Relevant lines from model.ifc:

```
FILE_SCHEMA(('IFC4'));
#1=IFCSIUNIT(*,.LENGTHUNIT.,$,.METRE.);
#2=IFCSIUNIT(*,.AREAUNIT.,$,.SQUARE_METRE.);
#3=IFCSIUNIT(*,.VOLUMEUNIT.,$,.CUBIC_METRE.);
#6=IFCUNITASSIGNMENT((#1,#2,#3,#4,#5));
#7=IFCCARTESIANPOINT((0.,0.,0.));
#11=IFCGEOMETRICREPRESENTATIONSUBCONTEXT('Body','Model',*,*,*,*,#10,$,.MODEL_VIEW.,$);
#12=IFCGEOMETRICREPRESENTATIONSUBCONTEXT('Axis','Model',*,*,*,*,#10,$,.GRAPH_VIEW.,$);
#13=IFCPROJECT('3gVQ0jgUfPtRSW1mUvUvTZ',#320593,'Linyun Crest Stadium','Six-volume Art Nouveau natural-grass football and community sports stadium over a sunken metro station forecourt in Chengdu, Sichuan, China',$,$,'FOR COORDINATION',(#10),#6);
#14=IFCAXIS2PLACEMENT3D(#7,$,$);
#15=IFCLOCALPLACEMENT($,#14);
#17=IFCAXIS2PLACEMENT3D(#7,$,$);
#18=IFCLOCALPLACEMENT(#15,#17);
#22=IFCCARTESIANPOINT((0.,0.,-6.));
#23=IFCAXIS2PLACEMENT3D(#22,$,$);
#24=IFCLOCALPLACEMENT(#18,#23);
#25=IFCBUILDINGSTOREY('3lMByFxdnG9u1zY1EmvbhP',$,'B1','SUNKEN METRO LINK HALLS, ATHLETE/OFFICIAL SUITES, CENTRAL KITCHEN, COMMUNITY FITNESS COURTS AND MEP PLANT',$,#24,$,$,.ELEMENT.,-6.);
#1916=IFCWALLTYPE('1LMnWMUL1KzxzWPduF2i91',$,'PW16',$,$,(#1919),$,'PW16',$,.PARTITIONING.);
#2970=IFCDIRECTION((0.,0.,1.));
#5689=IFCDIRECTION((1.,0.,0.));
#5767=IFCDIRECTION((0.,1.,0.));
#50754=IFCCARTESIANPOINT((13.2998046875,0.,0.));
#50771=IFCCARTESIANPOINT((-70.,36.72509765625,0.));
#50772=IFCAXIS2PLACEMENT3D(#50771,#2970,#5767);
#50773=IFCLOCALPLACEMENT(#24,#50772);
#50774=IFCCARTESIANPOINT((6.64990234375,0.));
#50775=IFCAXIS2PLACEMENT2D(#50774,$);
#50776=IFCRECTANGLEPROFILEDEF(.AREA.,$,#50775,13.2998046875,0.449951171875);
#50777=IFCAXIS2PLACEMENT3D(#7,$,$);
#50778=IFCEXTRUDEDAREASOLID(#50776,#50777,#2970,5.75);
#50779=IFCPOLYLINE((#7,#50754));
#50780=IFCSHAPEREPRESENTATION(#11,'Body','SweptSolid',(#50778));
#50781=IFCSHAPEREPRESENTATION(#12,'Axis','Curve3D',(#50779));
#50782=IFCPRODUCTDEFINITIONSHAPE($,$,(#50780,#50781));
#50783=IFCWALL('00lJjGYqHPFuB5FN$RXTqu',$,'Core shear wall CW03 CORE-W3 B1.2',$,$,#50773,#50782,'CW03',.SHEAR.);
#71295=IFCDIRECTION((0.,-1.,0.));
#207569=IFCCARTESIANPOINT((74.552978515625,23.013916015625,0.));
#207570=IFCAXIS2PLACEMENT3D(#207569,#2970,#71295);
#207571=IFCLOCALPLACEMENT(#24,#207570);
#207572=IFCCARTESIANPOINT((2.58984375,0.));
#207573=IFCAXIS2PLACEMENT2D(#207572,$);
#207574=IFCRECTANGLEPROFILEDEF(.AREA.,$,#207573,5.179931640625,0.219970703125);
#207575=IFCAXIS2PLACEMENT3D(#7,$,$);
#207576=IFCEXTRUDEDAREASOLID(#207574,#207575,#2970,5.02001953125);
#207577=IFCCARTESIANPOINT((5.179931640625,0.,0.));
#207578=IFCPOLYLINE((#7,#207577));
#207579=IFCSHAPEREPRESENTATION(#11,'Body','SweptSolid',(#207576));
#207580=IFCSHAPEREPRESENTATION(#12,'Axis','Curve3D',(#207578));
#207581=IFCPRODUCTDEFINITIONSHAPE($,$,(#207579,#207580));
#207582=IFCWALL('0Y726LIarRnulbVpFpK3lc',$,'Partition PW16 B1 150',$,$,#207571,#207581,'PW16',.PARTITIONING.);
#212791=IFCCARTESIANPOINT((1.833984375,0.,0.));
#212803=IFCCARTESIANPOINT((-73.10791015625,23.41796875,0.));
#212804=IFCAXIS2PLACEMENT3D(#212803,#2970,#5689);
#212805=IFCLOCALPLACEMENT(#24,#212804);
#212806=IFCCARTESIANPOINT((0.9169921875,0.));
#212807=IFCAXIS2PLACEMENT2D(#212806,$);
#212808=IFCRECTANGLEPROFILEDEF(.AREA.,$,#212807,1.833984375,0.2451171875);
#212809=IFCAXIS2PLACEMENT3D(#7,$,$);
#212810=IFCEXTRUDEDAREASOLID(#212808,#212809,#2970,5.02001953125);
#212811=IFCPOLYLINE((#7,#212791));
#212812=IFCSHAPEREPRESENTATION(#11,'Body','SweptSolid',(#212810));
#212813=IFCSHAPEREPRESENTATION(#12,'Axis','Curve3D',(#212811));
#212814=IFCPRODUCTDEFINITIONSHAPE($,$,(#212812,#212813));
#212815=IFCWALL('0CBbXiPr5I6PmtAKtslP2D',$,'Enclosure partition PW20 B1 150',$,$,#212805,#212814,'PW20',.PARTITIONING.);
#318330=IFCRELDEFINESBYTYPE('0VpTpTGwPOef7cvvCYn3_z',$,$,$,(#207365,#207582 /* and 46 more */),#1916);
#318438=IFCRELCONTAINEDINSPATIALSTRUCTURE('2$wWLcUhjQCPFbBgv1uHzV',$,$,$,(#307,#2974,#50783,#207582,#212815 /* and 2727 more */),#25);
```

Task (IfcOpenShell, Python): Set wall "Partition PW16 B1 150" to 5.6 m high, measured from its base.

```python
import ifcopenshell
import ifcopenshell.geom
import ifcopenshell.util.representation
import ifcopenshell.util.shape

model = ifcopenshell.open("model.ifc")
settings = ifcopenshell.geom.settings()


def volume(element):
    """Net volume in cubic metres, openings subtracted."""
    shape = ifcopenshell.geom.create_shape(settings, element)
    return ifcopenshell.util.shape.get_volume(shape.geometry)


wall = model.by_id(207582)
before = volume(wall)

body = ifcopenshell.util.representation.get_representation(wall, "Model", "Body")
solid = body.Items[0]
old_height = solid.Depth
solid.Depth = 5.6
after = volume(wall)

print(f"height {old_height:g} -> {solid.Depth:g}, volume {before:.3f} -> {after:.3f} m3")

model.write("model_v2.ifc")
```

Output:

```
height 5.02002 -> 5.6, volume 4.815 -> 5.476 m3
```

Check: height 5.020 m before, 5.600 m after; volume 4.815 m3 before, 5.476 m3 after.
